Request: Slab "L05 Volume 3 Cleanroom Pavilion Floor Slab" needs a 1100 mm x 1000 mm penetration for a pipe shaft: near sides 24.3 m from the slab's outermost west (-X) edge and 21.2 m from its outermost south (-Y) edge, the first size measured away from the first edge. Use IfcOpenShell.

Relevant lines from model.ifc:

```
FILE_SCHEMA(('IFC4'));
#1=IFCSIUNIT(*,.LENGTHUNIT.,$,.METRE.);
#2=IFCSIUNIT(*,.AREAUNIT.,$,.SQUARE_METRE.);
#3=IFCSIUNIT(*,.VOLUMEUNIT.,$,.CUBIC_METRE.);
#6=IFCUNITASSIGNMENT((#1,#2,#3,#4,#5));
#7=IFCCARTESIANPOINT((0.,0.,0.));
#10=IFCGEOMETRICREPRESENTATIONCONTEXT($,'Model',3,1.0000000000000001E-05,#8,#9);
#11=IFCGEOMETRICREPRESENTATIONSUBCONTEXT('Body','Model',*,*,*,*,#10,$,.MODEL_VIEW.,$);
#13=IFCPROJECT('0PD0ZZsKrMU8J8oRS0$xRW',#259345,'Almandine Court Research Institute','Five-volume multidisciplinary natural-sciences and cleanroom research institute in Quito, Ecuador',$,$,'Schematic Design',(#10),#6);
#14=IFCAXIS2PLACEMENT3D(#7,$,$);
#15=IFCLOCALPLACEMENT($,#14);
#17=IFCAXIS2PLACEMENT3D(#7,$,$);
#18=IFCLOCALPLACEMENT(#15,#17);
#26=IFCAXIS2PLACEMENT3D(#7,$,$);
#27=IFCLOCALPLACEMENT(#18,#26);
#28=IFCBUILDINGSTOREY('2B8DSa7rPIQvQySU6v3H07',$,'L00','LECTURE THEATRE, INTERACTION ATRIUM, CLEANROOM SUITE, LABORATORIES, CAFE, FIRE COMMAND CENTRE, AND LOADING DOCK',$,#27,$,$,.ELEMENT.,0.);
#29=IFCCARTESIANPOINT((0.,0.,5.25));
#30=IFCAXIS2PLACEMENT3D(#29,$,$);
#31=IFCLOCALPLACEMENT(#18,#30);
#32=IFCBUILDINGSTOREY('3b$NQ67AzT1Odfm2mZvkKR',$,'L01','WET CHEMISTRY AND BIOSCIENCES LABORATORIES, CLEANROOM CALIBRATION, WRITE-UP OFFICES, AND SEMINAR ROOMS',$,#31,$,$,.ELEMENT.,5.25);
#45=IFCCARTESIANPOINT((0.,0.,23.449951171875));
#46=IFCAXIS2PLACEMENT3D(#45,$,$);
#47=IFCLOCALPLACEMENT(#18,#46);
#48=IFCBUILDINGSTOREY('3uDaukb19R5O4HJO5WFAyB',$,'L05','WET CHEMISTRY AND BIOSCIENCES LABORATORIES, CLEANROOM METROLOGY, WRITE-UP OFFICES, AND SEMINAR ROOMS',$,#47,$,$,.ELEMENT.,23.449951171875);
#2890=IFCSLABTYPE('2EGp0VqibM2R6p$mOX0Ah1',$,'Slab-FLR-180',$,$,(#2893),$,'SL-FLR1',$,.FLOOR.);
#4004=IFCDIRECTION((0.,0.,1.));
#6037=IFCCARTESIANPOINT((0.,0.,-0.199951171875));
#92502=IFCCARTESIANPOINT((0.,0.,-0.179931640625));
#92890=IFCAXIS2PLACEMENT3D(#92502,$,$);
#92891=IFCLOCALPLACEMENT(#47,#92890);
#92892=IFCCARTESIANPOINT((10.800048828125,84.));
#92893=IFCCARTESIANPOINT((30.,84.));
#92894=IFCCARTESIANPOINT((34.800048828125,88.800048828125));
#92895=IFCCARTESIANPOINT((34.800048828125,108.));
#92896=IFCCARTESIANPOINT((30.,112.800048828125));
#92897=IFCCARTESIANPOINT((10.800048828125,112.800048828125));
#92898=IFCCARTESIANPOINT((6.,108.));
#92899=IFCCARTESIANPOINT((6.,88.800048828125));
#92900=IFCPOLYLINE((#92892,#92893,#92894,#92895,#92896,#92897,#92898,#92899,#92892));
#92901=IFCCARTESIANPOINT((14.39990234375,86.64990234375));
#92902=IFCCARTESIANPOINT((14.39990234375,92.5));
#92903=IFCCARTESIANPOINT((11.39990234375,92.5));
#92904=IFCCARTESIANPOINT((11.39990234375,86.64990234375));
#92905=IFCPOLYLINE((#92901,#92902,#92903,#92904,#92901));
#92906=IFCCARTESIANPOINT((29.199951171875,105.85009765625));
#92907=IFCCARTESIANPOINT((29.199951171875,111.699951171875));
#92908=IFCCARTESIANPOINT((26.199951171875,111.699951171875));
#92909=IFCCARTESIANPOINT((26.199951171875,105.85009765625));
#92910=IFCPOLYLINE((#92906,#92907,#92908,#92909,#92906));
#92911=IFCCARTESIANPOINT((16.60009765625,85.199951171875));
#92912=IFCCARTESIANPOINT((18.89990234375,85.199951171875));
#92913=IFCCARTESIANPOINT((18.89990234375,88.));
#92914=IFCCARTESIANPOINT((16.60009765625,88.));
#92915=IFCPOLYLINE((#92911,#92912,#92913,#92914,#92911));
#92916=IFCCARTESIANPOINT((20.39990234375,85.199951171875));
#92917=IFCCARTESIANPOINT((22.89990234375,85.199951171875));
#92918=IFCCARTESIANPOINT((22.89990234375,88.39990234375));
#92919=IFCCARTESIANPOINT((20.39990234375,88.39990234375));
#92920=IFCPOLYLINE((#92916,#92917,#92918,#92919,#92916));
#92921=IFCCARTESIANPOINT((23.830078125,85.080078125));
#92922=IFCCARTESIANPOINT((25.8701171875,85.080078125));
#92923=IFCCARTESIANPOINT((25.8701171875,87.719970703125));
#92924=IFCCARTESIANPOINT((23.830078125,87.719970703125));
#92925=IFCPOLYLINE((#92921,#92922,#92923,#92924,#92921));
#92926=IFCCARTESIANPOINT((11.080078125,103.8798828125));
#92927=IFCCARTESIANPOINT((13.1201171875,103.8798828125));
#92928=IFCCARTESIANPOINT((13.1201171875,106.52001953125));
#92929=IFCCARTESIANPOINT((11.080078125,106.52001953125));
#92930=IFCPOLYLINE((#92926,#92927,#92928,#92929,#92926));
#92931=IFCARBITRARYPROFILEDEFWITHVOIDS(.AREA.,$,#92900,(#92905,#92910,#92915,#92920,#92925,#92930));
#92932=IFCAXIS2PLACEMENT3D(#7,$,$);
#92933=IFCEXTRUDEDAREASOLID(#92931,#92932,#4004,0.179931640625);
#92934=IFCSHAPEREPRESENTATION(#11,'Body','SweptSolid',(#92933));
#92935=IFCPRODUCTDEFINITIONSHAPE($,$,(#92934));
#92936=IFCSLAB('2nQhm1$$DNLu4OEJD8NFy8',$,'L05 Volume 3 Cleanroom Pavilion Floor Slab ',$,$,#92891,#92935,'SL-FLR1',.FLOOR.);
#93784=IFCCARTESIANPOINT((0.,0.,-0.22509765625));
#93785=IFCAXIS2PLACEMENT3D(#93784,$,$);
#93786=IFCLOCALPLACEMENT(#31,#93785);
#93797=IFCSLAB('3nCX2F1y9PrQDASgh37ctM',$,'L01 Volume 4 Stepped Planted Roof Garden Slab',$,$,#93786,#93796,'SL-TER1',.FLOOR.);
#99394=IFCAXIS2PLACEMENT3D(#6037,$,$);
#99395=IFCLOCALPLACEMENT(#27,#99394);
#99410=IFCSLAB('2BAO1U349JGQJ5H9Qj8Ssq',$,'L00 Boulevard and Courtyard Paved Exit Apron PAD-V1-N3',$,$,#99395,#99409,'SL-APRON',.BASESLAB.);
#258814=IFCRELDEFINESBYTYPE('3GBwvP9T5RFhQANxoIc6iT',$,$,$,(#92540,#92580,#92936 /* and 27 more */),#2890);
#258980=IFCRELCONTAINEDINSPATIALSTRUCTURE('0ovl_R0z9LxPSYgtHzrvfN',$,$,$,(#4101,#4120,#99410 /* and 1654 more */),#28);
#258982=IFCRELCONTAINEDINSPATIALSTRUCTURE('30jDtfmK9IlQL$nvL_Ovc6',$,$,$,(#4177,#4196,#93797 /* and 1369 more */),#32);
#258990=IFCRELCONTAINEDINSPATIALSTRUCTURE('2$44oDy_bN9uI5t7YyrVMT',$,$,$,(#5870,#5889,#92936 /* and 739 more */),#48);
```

```python
import numpy as np
import ifcopenshell
import ifcopenshell.api.feature
import ifcopenshell.api.geometry
import ifcopenshell.api.root
import ifcopenshell.geom
import ifcopenshell.util.placement
import ifcopenshell.util.representation
import ifcopenshell.util.shape
import ifcopenshell.util.unit

model = ifcopenshell.open("model.ifc")
unit_scale = ifcopenshell.util.unit.calculate_unit_scale(model)
settings = ifcopenshell.geom.settings()


def volume(element):
    """Net volume in cubic metres, openings subtracted."""
    shape = ifcopenshell.geom.create_shape(settings, element)
    return ifcopenshell.util.shape.get_volume(shape.geometry)


slab = model.by_id(92936)
before = volume(slab)

# Extent in the slab's own axes, in metres. The edges named are its -X and -Y sides.
slab_shape = ifcopenshell.geom.create_shape(settings, slab)
vertices = ifcopenshell.util.shape.get_vertices(slab_shape.geometry)
x_min, y_min, bottom = vertices.min(axis=0)
top = vertices[:, 2].max()

opening = ifcopenshell.api.root.create_entity(model, ifc_class="IfcOpeningElement", name="Pipe shaft opening", predefined_type="OPENING")
context = ifcopenshell.util.representation.get_context(model, "Model", "Body", "MODEL_VIEW")
width, depth = 1.1, 1
outline = [(0.0, 0.0), (width, 0.0), (width, depth), (0.0, depth), (0.0, 0.0)]
# Overshoot both faces by 50 mm so the cut is clean.
shape = ifcopenshell.api.geometry.add_slab_representation(
    model, context=context, depth=top - bottom + 0.1, polyline=outline
)
ifcopenshell.api.geometry.assign_representation(model, product=opening, representation=shape)

matrix = ifcopenshell.util.placement.get_local_placement(slab.ObjectPlacement)
matrix[:, 3] = matrix @ np.append(np.array([x_min + 24.3, y_min + 21.2, bottom - 0.05]) / unit_scale, 1.0)
ifcopenshell.api.geometry.edit_object_placement(model, product=opening, matrix=matrix, is_si=False)
ifcopenshell.api.feature.add_feature(model, feature=opening, element=slab)

after = volume(slab)

print(f"slab volume {before:.3f} -> {after:.3f} m3")

model.write("model_updated.ifc")
```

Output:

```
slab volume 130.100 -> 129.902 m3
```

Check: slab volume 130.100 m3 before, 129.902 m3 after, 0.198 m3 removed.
